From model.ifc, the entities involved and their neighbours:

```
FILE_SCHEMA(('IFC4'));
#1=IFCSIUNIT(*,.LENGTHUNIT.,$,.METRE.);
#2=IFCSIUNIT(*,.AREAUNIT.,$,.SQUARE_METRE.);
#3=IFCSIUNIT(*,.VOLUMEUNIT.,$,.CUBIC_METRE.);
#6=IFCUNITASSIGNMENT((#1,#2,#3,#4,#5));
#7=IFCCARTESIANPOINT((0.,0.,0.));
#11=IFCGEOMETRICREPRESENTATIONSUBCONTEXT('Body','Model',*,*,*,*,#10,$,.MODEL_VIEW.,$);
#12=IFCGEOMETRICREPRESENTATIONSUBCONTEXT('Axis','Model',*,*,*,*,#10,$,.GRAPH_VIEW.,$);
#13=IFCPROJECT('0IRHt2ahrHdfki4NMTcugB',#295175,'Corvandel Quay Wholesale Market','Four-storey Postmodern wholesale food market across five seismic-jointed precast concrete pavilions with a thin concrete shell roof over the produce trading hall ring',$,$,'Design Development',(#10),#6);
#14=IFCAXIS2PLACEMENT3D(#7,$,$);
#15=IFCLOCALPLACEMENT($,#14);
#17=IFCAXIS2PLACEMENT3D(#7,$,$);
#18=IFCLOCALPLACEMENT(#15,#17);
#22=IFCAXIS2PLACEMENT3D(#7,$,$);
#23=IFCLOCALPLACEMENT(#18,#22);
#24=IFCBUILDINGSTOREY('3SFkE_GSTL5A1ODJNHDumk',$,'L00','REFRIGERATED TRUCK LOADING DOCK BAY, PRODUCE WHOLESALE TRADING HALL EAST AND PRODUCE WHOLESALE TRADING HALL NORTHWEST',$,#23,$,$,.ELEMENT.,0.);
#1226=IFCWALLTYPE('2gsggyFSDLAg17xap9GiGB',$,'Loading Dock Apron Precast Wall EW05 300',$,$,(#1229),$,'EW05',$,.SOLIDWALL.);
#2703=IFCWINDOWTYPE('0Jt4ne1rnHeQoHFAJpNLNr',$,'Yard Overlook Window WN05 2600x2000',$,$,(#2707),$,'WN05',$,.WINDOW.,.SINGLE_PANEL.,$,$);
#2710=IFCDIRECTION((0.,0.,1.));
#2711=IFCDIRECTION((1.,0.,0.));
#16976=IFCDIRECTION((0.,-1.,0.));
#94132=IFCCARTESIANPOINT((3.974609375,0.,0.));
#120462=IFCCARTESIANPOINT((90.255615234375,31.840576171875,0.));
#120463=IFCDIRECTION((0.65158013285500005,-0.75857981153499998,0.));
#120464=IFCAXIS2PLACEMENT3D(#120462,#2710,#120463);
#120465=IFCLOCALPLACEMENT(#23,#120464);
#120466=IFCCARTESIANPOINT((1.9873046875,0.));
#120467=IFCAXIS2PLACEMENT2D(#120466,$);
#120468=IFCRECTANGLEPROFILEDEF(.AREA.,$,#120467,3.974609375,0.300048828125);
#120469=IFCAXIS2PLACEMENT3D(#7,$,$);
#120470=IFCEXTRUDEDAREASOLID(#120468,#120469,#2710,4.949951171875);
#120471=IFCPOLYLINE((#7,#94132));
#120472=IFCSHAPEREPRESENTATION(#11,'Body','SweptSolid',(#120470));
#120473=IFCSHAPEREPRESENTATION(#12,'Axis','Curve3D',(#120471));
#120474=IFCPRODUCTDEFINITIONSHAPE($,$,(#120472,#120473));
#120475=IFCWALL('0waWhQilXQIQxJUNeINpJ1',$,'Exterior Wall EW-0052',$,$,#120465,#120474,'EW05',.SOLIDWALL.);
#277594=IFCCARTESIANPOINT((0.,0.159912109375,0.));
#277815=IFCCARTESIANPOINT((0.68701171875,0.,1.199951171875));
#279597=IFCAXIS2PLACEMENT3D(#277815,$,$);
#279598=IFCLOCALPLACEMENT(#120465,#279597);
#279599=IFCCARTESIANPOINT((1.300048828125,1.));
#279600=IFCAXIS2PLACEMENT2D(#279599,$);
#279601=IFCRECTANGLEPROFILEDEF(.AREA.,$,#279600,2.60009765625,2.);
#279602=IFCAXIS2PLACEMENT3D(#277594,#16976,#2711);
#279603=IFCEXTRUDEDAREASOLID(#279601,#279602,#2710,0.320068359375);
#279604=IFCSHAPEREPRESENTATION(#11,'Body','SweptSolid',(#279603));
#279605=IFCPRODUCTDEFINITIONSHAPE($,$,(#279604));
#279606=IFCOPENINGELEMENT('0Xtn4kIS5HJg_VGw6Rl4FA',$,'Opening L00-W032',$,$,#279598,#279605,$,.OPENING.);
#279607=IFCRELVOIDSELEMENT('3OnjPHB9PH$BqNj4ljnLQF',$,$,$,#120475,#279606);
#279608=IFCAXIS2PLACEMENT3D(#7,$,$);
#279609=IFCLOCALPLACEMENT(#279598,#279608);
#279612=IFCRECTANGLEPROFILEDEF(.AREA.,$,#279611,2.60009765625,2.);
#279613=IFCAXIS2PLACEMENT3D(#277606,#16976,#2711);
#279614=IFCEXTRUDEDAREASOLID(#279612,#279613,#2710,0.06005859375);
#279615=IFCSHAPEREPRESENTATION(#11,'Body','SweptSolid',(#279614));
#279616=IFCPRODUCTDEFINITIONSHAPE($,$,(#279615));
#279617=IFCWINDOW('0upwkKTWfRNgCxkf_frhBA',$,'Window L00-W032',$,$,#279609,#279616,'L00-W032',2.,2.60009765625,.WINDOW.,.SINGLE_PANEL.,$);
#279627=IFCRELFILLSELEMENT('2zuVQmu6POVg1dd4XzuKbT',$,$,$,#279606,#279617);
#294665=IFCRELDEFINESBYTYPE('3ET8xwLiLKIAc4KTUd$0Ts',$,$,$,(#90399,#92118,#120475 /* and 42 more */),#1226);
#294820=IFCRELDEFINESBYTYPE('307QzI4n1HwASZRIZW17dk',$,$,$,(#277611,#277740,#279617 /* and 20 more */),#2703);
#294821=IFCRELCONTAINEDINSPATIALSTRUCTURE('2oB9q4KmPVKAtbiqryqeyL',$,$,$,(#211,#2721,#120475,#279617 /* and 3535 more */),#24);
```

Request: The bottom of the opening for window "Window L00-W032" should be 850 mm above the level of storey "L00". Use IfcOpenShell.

```python
import numpy as np
import ifcopenshell
import ifcopenshell.api.geometry
import ifcopenshell.geom
import ifcopenshell.util.element
import ifcopenshell.util.placement
import ifcopenshell.util.shape
import ifcopenshell.util.unit

model = ifcopenshell.open("model.ifc")
unit_scale = ifcopenshell.util.unit.calculate_unit_scale(model)

window = model.by_id(279617)
opening = window.FillsVoids[0].RelatingOpeningElement
storey = ifcopenshell.util.element.get_container(window, ifc_class="IfcBuildingStorey")
level = ifcopenshell.util.placement.get_local_placement(storey.ObjectPlacement)[2, 3]

# The opening's origin need not be at the sill, so measure its lowest point.
shape = ifcopenshell.geom.create_shape(ifcopenshell.geom.settings(), opening)
bottom = ifcopenshell.util.shape.get_shape_bottom_elevation(shape, shape.geometry) / unit_scale
dz = level + 0.85 / unit_scale - bottom

shift = np.array([0.0, 0.0, dz])
# The window is placed relative to its opening, so it follows when the opening moves.
matrix = ifcopenshell.util.placement.get_local_placement(opening.ObjectPlacement)
matrix[:3, 3] += shift
ifcopenshell.api.geometry.edit_object_placement(
    model, product=opening, matrix=matrix, is_si=False, should_transform_children=True
)

print(f"moved by {dz * unit_scale:+.3f} m")

model.write("model_updated.ifc")
```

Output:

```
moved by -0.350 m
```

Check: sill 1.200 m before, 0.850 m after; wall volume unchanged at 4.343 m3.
